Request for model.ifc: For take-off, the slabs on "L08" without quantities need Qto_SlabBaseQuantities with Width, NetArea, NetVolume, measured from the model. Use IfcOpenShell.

First a look at what the model holds.

```python
import ifcopenshell
import ifcopenshell.util.element
import ifcopenshell.util.unit

model = ifcopenshell.open("model.ifc")
print(model.schema)
for unit_type in ("LENGTHUNIT", "AREAUNIT", "VOLUMEUNIT"):
    print(unit_type, ifcopenshell.util.unit.calculate_unit_scale(model, unit_type))
storey = next(s for s in model.by_type("IfcBuildingStorey") if s.Name == "L08")
slabs = [e for e in ifcopenshell.util.element.get_decomposition(storey) if e.is_a("IfcSlab")]
for e in sorted(slabs, key=lambda e: e.id()):
    print(e.id(), e.is_a(), e.Name, list(ifcopenshell.util.element.get_psets(e, qtos_only=True)), sep=" | ")
```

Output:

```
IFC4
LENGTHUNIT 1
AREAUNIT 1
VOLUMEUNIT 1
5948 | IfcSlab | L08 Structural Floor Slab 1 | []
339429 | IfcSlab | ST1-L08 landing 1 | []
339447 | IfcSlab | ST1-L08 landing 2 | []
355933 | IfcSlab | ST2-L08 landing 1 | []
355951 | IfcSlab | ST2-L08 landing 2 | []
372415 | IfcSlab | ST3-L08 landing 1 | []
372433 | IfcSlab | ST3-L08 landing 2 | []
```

```python
import ifcopenshell
import ifcopenshell.api.pset
import ifcopenshell.geom
import ifcopenshell.util.element
import ifcopenshell.util.shape
import ifcopenshell.util.unit

model = ifcopenshell.open("model.ifc")
unit_scale = ifcopenshell.util.unit.calculate_unit_scale(model)
area_scale = ifcopenshell.util.unit.calculate_unit_scale(model, "AREAUNIT")
volume_scale = ifcopenshell.util.unit.calculate_unit_scale(model, "VOLUMEUNIT")
settings = ifcopenshell.geom.settings()

storey = next(s for s in model.by_type("IfcBuildingStorey") if s.Name == "L08")
slabs = [e for e in ifcopenshell.util.element.get_decomposition(storey) if e.is_a("IfcSlab")]

for e in sorted(slabs, key=lambda e: e.id()):
    if ifcopenshell.util.element.get_psets(e, qtos_only=True, should_inherit=False):
        continue
    # Geometry comes back in metres, in the element's own axes.
    shape = ifcopenshell.geom.create_shape(settings, e)
    values = {
        "Width": ifcopenshell.util.shape.get_z(shape.geometry) / unit_scale,
        "NetArea": ifcopenshell.util.shape.get_footprint_area(shape.geometry) / area_scale,
        "NetVolume": ifcopenshell.util.shape.get_volume(shape.geometry) / volume_scale,
    }
    qto = ifcopenshell.api.pset.add_qto(model, product=e, name="Qto_SlabBaseQuantities")
    ifcopenshell.api.pset.edit_qto(model, qto=qto, properties=values)
    print(e.id(), {k: round(v, 3) for k, v in values.items()})

model.write("model_edited.ifc")
```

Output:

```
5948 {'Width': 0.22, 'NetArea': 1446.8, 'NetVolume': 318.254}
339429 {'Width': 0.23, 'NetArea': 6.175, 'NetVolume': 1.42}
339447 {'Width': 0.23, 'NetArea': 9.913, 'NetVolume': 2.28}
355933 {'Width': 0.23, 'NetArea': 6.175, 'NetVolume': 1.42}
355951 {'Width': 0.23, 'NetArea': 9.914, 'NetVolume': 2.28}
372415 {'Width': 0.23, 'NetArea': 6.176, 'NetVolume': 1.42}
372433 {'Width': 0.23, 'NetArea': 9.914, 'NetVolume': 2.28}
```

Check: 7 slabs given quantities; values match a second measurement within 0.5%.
